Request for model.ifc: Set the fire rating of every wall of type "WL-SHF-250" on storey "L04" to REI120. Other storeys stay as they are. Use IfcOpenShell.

First a look at what the model holds.

```python
import ifcopenshell
import ifcopenshell.util.element

model = ifcopenshell.open("model.ifc")
print(model.schema)
storey = next(s for s in model.by_type("IfcBuildingStorey") if s.Name == "L04")
walls = [e for e in ifcopenshell.util.element.get_decomposition(storey) if e.is_a("IfcWall")]
seen = {}
for e in walls:
    element_type = ifcopenshell.util.element.get_type(e)
    key = (element_type.Name if element_type != e and element_type else None, ifcopenshell.util.element.get_pset(e, "Pset_WallCommon", "FireRating"))
    seen[key] = seen.get(key, 0) + 1
for (name, value), count in sorted(seen.items(), key=str):
    print(count, "x", name, "|", value)
```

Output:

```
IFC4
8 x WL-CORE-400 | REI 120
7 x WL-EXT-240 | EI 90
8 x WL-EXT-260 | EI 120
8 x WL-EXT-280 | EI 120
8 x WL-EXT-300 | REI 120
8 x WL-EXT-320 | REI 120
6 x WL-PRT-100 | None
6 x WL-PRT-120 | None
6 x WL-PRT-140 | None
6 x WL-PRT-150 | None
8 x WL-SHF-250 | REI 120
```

```python
import ifcopenshell
import ifcopenshell.api.pset
import ifcopenshell.util.element

model = ifcopenshell.open("model.ifc")

storey = next(s for s in model.by_type("IfcBuildingStorey") if s.Name == "L04")
walls = [e for e in ifcopenshell.util.element.get_decomposition(storey) if e.is_a("IfcWall")]

count = 0
for e in walls:
    element_type = ifcopenshell.util.element.get_type(e)
    if element_type in (None, e) or element_type.Name != "WL-SHF-250":
        continue
    # add_pset returns the element's existing set when there is one.
    pset = ifcopenshell.api.pset.add_pset(model, product=e, name="Pset_WallCommon")
    ifcopenshell.api.pset.edit_pset(model, pset=pset, properties={"FireRating": "REI120"})
    count += 1

print(count, "walls updated")

model.write("model_updated.ifc")
```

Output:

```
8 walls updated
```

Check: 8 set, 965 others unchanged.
